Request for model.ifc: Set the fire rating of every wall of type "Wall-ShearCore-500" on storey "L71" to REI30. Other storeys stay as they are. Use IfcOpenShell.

First a look at what the model holds.

```python
import ifcopenshell
import ifcopenshell.util.element

model = ifcopenshell.open("model.ifc")
print(model.schema)
storey = next(s for s in model.by_type("IfcBuildingStorey") if s.Name == "L71")
walls = [e for e in ifcopenshell.util.element.get_decomposition(storey) if e.is_a("IfcWall")]
seen = {}
for e in walls:
    element_type = ifcopenshell.util.element.get_type(e)
    key = (element_type.Name if element_type != e and element_type else None, ifcopenshell.util.element.get_pset(e, "Pset_WallCommon", "FireRating"))
    seen[key] = seen.get(key, 0) + 1
for (name, value), count in sorted(seen.items(), key=str):
    print(count, "x", name, "|", value)
```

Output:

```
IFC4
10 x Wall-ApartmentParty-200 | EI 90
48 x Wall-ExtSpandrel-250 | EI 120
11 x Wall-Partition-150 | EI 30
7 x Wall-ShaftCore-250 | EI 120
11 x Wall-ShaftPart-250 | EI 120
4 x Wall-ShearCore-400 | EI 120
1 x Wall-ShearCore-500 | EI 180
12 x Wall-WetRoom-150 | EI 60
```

```python
import ifcopenshell
import ifcopenshell.api.pset
import ifcopenshell.util.element

model = ifcopenshell.open("model.ifc")

storey = next(s for s in model.by_type("IfcBuildingStorey") if s.Name == "L71")
walls = [e for e in ifcopenshell.util.element.get_decomposition(storey) if e.is_a("IfcWall")]

count = 0
for e in walls:
    element_type = ifcopenshell.util.element.get_type(e)
    if element_type in (None, e) or element_type.Name != "Wall-ShearCore-500":
        continue
    found = ifcopenshell.util.element.get_pset(e, "Pset_WallCommon", should_inherit=False)
    if found:
        pset = model.by_id(found["id"])
        if len(ifcopenshell.util.element.get_elements_by_pset(pset)) > 1:
            pset = ifcopenshell.api.pset.unshare_pset(model, products=[e], pset=pset)[0]
    else:
        pset = ifcopenshell.api.pset.add_pset(model, product=e, name="Pset_WallCommon")
    ifcopenshell.api.pset.edit_pset(model, pset=pset, properties={"FireRating": "REI30"})
    count += 1

print(count, "walls updated")

model.write("model_v2.ifc")
```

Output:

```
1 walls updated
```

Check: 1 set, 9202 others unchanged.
